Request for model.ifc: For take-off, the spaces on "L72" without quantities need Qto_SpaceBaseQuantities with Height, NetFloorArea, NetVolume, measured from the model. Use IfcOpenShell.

First a look at what the model holds.

```python
import ifcopenshell
import ifcopenshell.util.element
import ifcopenshell.util.unit

model = ifcopenshell.open("model.ifc")
print(model.schema)
for unit_type in ("LENGTHUNIT", "AREAUNIT", "VOLUMEUNIT"):
    print(unit_type, ifcopenshell.util.unit.calculate_unit_scale(model, unit_type))
storey = next(s for s in model.by_type("IfcBuildingStorey") if s.Name == "L72")
spaces = [e for e in ifcopenshell.util.element.get_decomposition(storey) if e.is_a("IfcSpace")]
for e in sorted(spaces, key=lambda e: e.id()):
    print(e.id(), e.is_a(), e.Name, list(ifcopenshell.util.element.get_psets(e, qtos_only=True)), sep=" | ")
```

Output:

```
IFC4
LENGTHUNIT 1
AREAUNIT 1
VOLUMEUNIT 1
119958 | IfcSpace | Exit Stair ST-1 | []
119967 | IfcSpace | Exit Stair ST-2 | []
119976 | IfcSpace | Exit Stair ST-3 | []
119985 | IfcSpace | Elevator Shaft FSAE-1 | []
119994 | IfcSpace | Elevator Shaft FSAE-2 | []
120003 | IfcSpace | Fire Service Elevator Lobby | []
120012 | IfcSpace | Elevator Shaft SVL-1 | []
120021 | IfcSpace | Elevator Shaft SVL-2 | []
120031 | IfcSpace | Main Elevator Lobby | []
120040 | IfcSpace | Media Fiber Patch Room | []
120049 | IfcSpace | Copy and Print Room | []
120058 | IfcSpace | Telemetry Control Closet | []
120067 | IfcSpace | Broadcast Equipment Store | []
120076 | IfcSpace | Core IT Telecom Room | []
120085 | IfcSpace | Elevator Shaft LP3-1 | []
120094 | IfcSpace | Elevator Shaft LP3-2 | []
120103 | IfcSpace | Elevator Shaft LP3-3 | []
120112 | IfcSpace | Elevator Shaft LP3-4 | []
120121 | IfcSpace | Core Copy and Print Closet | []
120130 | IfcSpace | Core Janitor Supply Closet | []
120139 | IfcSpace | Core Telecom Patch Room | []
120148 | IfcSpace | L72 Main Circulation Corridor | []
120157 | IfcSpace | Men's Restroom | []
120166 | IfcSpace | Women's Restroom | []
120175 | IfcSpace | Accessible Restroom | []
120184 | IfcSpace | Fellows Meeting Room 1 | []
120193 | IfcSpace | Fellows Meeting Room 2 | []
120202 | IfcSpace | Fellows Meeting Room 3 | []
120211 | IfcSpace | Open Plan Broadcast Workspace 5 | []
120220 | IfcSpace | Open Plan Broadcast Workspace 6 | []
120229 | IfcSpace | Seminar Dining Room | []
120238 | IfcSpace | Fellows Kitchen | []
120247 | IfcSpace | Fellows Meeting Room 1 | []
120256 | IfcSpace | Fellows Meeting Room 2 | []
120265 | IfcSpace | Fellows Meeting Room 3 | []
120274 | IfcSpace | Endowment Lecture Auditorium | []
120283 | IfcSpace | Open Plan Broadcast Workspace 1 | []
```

```python
import ifcopenshell
import ifcopenshell.api.pset
import ifcopenshell.geom
import ifcopenshell.util.element
import ifcopenshell.util.shape
import ifcopenshell.util.unit

model = ifcopenshell.open("model.ifc")
unit_scale = ifcopenshell.util.unit.calculate_unit_scale(model)
area_scale = ifcopenshell.util.unit.calculate_unit_scale(model, "AREAUNIT")
volume_scale = ifcopenshell.util.unit.calculate_unit_scale(model, "VOLUMEUNIT")
settings = ifcopenshell.geom.settings()

storey = next(s for s in model.by_type("IfcBuildingStorey") if s.Name == "L72")
spaces = [e for e in ifcopenshell.util.element.get_decomposition(storey) if e.is_a("IfcSpace")]

for e in sorted(spaces, key=lambda e: e.id()):
    if ifcopenshell.util.element.get_psets(e, qtos_only=True, should_inherit=False):
        continue
    # Geometry comes back in metres, in the element's own axes.
    shape = ifcopenshell.geom.create_shape(settings, e)
    values = {
        "Height": ifcopenshell.util.shape.get_z(shape.geometry) / unit_scale,
        "NetFloorArea": ifcopenshell.util.shape.get_footprint_area(shape.geometry) / area_scale,
        "NetVolume": ifcopenshell.util.shape.get_volume(shape.geometry) / volume_scale,
    }
    qto = ifcopenshell.api.pset.add_qto(model, product=e, name="Qto_SpaceBaseQuantities")
    ifcopenshell.api.pset.edit_qto(model, qto=qto, properties=values)
    print(e.id(), {k: round(v, 3) for k, v in values.items()})

model.write("model_v2.ifc")
```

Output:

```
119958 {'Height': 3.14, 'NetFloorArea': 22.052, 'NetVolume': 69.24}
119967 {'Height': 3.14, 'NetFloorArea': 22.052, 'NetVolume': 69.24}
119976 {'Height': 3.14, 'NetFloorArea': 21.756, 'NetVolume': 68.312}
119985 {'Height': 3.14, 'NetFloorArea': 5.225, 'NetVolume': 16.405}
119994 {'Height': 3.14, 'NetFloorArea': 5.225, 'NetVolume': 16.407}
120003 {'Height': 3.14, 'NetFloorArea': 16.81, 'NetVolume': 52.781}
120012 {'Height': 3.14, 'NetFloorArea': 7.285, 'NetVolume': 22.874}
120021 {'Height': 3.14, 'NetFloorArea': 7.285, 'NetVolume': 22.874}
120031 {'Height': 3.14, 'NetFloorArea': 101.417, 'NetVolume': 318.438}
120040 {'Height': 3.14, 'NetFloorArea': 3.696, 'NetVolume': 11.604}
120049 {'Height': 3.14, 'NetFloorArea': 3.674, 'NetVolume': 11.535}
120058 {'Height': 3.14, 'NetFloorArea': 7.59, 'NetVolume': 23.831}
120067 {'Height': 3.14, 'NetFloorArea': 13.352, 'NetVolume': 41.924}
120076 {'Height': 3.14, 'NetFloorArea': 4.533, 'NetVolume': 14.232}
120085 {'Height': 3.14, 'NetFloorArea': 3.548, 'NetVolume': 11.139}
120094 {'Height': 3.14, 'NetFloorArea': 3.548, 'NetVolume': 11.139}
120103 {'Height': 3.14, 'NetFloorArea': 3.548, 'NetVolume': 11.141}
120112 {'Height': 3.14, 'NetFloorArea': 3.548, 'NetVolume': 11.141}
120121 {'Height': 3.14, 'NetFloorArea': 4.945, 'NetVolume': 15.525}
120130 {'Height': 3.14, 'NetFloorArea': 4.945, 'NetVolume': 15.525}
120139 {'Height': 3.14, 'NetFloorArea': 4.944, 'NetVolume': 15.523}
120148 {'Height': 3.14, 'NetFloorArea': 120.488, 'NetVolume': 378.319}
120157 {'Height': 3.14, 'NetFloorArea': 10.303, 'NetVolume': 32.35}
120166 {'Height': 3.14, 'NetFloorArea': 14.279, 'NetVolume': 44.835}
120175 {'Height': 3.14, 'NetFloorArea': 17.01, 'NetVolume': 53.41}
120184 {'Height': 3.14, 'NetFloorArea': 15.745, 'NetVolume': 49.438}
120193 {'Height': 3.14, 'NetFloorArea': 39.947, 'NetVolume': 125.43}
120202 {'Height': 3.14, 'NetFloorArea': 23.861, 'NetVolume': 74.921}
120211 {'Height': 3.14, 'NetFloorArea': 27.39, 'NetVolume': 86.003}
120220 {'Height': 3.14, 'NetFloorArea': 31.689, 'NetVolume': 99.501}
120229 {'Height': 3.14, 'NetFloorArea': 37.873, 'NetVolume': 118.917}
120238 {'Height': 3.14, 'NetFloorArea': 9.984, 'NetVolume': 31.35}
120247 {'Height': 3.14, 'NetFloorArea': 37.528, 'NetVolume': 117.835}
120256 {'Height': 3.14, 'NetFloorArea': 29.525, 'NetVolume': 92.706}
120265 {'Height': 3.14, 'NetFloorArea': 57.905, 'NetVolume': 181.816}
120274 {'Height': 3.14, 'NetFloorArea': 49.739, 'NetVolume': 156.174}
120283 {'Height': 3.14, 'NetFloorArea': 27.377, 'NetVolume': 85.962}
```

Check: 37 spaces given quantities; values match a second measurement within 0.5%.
